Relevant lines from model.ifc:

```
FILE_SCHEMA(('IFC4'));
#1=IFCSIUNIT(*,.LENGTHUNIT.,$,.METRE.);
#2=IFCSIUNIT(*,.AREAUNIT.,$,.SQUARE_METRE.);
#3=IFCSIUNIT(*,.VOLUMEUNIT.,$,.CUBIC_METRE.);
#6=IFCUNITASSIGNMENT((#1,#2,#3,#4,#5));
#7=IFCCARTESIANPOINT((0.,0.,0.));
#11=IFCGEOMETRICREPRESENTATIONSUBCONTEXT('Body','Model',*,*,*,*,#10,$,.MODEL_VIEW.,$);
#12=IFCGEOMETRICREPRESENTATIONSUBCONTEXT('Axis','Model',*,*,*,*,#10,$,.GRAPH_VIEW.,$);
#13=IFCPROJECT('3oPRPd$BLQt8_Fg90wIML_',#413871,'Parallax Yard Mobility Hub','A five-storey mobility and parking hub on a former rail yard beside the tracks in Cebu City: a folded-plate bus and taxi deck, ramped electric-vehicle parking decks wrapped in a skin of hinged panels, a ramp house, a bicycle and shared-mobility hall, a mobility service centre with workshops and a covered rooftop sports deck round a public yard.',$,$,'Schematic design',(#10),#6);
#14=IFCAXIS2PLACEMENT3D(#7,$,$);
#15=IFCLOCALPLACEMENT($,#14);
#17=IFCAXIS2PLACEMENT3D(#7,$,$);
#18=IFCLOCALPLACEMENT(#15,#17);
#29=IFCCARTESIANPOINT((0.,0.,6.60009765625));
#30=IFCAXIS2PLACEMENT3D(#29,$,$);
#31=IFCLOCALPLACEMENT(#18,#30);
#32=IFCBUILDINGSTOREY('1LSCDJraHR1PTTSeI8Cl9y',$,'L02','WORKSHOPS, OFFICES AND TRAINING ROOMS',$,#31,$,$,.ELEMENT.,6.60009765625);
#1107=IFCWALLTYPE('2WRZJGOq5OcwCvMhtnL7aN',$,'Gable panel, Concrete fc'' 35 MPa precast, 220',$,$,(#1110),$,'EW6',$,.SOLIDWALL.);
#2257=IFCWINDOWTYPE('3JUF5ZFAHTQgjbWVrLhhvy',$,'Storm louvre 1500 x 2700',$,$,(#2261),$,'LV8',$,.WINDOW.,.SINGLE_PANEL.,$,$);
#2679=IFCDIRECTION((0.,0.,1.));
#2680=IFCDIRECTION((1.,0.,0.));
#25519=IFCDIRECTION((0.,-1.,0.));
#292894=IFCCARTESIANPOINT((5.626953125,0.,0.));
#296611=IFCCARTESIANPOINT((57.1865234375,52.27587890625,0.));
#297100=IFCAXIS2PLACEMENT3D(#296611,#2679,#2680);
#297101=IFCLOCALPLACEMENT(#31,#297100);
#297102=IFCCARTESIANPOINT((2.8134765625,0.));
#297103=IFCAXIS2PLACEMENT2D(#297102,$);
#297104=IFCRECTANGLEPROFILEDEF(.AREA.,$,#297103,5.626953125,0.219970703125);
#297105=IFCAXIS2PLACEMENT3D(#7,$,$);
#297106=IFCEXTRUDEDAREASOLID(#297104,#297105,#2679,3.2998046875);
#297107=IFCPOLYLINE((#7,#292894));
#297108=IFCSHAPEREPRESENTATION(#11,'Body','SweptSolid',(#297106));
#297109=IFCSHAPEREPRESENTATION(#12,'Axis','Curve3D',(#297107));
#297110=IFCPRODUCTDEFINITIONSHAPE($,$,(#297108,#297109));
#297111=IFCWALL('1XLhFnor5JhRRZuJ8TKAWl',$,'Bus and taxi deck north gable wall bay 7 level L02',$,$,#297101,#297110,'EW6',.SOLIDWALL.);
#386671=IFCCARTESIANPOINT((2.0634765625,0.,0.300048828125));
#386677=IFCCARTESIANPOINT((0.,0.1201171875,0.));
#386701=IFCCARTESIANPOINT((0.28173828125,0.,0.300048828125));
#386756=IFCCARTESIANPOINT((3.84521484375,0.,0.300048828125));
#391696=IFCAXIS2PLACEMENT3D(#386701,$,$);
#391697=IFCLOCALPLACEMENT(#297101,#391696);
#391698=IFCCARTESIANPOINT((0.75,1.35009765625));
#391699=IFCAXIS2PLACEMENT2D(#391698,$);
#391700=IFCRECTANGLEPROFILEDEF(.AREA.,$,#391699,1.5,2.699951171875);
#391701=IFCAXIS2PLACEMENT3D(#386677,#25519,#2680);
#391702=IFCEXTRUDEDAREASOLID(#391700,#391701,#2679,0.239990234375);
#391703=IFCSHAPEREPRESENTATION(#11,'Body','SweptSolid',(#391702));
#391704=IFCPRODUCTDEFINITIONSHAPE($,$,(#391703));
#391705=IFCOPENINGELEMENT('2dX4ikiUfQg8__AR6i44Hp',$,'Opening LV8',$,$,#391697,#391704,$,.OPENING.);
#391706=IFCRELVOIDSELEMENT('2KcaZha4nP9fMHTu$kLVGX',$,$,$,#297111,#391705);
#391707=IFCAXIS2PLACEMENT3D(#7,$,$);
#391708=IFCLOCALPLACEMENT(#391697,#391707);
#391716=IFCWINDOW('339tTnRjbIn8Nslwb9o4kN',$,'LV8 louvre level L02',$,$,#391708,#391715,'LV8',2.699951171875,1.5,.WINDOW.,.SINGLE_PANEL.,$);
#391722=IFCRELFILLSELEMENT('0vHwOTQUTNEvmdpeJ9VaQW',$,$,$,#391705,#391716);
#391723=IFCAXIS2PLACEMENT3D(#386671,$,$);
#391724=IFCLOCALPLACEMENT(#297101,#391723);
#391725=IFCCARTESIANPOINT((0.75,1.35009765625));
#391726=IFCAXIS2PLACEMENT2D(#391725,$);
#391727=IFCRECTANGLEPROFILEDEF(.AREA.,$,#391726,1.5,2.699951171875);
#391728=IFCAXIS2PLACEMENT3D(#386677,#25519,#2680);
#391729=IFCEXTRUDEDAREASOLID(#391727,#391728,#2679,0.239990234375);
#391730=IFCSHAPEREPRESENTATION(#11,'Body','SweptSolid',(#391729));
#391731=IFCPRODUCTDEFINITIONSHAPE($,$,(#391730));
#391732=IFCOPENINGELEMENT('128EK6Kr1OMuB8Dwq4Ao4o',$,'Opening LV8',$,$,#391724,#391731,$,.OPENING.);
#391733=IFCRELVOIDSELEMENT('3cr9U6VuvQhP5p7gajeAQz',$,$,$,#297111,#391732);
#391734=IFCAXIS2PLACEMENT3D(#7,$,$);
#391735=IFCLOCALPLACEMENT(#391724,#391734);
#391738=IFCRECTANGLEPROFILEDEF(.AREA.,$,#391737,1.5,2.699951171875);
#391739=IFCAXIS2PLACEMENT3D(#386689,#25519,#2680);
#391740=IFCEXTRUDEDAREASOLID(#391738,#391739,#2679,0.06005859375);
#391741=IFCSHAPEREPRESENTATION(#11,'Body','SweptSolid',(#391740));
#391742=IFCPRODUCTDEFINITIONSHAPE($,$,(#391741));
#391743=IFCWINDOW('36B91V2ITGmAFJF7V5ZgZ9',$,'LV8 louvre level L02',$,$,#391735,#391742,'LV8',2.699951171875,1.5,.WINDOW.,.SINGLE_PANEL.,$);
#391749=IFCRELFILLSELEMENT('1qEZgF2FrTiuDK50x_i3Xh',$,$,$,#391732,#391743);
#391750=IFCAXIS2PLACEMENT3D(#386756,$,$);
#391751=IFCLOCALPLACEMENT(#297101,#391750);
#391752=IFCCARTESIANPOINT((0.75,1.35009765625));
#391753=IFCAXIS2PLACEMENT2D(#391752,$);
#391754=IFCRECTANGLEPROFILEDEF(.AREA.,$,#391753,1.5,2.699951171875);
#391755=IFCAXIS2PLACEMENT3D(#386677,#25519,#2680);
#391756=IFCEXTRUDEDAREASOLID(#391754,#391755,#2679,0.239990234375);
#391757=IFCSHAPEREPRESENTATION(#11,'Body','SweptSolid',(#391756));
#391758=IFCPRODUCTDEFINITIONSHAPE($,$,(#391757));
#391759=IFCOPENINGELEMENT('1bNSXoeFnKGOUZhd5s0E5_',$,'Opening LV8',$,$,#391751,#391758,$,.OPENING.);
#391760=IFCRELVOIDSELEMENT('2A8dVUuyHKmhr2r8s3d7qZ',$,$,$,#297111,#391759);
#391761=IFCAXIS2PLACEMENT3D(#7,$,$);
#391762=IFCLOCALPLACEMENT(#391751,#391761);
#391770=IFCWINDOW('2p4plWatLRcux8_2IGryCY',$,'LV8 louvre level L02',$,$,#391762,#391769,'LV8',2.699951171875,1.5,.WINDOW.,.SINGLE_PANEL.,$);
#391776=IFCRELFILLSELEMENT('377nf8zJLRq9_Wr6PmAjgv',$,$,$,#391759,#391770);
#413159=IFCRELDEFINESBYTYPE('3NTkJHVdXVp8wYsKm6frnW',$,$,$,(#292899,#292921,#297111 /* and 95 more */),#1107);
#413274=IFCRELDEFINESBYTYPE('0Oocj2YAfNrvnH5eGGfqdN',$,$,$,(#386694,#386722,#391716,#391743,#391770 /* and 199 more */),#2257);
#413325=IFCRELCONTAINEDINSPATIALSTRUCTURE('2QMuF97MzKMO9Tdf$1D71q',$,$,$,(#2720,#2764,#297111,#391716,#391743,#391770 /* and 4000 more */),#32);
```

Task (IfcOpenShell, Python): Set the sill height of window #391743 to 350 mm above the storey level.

```python
import numpy as np
import ifcopenshell
import ifcopenshell.api.geometry
import ifcopenshell.geom
import ifcopenshell.util.element
import ifcopenshell.util.placement
import ifcopenshell.util.shape
import ifcopenshell.util.unit

model = ifcopenshell.open("model.ifc")
unit_scale = ifcopenshell.util.unit.calculate_unit_scale(model)

window = model.by_guid("36B91V2ITGmAFJF7V5ZgZ9")
opening = window.FillsVoids[0].RelatingOpeningElement
storey = ifcopenshell.util.element.get_container(window, ifc_class="IfcBuildingStorey")
level = ifcopenshell.util.placement.get_local_placement(storey.ObjectPlacement)[2, 3]

# The opening's origin need not be at the sill, so measure its lowest point.
shape = ifcopenshell.geom.create_shape(ifcopenshell.geom.settings(), opening)
bottom = ifcopenshell.util.shape.get_shape_bottom_elevation(shape, shape.geometry) / unit_scale
dz = level + 0.35 - bottom

shift = np.array([0.0, 0.0, dz])
# The window is placed relative to its opening, so it follows when the opening moves.
matrix = ifcopenshell.util.placement.get_local_placement(opening.ObjectPlacement)
matrix[:3, 3] += shift
ifcopenshell.api.geometry.edit_object_placement(
    model, product=opening, matrix=matrix, is_si=False, should_transform_children=True
)

print(f"moved by {dz * unit_scale:+.3f} m")

model.write("model_rev.ifc")
```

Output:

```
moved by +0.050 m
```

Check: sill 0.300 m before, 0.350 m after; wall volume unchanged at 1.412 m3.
